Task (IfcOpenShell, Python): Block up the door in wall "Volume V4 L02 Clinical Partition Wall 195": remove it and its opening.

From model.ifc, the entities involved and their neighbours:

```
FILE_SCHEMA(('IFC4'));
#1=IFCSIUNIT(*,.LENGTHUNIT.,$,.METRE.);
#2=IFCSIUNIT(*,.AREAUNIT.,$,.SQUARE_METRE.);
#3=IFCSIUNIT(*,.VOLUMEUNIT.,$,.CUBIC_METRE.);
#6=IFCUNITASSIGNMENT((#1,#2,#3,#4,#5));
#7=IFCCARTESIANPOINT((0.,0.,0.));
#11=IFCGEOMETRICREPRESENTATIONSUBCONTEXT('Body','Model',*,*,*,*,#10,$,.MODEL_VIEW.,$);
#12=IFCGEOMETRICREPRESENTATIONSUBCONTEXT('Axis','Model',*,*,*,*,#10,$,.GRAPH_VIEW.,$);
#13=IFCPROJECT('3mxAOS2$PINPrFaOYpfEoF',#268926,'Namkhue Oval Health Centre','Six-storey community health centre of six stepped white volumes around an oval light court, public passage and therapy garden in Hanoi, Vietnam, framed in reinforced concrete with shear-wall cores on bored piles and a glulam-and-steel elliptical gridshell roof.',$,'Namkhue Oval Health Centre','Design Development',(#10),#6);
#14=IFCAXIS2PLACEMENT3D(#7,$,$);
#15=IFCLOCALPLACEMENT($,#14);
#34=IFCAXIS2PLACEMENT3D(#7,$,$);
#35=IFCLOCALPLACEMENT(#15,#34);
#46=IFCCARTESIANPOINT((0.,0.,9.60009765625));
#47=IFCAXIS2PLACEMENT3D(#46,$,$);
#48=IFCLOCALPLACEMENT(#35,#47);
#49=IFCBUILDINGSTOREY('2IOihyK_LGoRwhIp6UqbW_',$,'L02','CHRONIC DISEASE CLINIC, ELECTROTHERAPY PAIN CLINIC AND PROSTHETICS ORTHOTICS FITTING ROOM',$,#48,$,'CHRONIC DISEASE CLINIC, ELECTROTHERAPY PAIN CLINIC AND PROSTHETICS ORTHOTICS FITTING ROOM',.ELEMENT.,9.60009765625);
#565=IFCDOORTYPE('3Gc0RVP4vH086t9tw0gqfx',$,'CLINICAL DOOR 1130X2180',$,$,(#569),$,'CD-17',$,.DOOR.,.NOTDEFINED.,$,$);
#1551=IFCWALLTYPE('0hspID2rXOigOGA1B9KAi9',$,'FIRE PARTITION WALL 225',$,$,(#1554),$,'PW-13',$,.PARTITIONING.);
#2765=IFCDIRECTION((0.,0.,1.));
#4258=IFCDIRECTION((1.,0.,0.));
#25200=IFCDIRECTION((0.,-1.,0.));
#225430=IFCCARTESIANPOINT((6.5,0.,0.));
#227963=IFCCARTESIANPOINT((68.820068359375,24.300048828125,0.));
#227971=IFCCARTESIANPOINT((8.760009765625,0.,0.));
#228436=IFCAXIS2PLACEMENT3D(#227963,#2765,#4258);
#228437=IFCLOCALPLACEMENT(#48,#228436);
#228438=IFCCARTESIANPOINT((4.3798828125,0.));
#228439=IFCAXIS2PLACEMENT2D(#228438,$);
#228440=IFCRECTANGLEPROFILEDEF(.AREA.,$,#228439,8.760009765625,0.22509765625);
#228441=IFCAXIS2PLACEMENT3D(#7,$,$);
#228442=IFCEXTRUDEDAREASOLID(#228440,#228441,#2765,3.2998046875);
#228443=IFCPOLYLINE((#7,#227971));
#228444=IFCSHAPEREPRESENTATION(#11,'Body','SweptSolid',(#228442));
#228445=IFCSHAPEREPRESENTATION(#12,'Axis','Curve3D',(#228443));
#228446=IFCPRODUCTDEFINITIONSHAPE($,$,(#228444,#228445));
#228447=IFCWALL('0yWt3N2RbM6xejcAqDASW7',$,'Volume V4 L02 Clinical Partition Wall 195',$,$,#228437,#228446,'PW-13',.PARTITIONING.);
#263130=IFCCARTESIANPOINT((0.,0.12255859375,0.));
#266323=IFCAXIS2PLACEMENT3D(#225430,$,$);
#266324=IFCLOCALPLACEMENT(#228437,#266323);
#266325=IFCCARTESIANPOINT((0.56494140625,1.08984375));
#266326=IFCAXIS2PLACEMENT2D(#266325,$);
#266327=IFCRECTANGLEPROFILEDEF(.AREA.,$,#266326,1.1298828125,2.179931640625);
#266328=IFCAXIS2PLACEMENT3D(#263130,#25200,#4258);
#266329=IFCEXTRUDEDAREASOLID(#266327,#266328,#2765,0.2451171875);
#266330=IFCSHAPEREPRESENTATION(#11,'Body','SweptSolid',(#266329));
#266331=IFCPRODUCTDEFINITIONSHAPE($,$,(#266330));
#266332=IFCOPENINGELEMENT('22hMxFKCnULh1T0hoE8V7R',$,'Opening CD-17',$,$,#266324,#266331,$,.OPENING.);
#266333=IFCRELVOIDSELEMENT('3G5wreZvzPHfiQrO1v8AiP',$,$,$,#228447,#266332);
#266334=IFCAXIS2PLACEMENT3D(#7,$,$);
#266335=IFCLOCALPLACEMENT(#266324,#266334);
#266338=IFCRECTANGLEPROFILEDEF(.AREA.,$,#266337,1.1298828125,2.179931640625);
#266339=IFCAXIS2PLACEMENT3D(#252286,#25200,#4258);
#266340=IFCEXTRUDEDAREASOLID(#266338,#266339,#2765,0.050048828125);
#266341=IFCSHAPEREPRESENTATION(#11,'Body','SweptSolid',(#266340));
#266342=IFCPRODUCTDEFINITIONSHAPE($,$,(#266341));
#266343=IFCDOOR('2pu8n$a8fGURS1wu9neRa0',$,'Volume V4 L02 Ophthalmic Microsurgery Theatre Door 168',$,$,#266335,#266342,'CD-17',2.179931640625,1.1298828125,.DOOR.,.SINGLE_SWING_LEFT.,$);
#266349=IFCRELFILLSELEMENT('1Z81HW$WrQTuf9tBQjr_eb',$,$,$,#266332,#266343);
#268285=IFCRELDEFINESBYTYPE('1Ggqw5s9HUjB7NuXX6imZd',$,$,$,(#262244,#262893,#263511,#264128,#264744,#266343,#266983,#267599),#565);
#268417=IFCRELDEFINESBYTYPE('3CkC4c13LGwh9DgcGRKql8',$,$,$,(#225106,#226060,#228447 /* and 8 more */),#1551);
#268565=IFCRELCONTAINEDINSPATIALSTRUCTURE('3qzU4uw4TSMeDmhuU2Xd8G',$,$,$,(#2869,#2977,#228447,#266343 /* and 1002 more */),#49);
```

```python
import ifcopenshell
import ifcopenshell.api.feature
import ifcopenshell.api.root
import ifcopenshell.geom
import ifcopenshell.util.shape

model = ifcopenshell.open("model.ifc")
settings = ifcopenshell.geom.settings()


def volume(element):
    """Net volume in cubic metres, openings subtracted."""
    shape = ifcopenshell.geom.create_shape(settings, element)
    return ifcopenshell.util.shape.get_volume(shape.geometry)


door = model.by_id(266343)
opening = door.FillsVoids[0].RelatingOpeningElement
wall = opening.VoidsElements[0].RelatingBuildingElement
before = volume(wall)

ifcopenshell.api.root.remove_product(model, product=door)
ifcopenshell.api.feature.remove_feature(model, feature=opening)

after = volume(wall)

print(f"wall volume {before:.3f} -> {after:.3f} m3")

model.write("model_v2.ifc")
```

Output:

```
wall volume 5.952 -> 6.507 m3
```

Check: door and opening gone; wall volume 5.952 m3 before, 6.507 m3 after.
